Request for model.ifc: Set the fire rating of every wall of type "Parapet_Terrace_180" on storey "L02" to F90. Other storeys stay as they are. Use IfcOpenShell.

First a look at what the model holds.

```python
import ifcopenshell
import ifcopenshell.util.element

model = ifcopenshell.open("model.ifc")
print(model.schema)
storey = next(s for s in model.by_type("IfcBuildingStorey") if s.Name == "L02")
walls = [e for e in ifcopenshell.util.element.get_decomposition(storey) if e.is_a("IfcWall")]
seen = {}
for e in walls:
    element_type = ifcopenshell.util.element.get_type(e)
    key = (element_type.Name if element_type != e and element_type else None, ifcopenshell.util.element.get_pset(e, "Pset_WallCommon", "FireRating"))
    seen[key] = seen.get(key, 0) + 1
for (name, value), count in sorted(seen.items(), key=str):
    print(count, "x", name, "|", value)
```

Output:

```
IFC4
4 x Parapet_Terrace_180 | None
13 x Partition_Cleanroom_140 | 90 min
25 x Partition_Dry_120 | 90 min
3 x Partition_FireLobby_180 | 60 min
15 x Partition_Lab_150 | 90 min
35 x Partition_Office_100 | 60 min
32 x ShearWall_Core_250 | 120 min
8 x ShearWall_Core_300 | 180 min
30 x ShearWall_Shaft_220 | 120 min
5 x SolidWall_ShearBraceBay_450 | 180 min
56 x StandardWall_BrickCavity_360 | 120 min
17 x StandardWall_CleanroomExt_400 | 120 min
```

```python
import ifcopenshell
import ifcopenshell.api.pset
import ifcopenshell.util.element

model = ifcopenshell.open("model.ifc")

storey = next(s for s in model.by_type("IfcBuildingStorey") if s.Name == "L02")
walls = [e for e in ifcopenshell.util.element.get_decomposition(storey) if e.is_a("IfcWall")]

count = 0
for e in walls:
    element_type = ifcopenshell.util.element.get_type(e)
    if element_type in (None, e) or element_type.Name != "Parapet_Terrace_180":
        continue
    # add_pset returns the element's existing set when there is one.
    pset = ifcopenshell.api.pset.add_pset(model, product=e, name="Pset_WallCommon")
    ifcopenshell.api.pset.edit_pset(model, pset=pset, properties={"FireRating": "F90"})
    count += 1

print(count, "walls updated")

model.write("model_edited.ifc")
```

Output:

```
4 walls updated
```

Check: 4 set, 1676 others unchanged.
